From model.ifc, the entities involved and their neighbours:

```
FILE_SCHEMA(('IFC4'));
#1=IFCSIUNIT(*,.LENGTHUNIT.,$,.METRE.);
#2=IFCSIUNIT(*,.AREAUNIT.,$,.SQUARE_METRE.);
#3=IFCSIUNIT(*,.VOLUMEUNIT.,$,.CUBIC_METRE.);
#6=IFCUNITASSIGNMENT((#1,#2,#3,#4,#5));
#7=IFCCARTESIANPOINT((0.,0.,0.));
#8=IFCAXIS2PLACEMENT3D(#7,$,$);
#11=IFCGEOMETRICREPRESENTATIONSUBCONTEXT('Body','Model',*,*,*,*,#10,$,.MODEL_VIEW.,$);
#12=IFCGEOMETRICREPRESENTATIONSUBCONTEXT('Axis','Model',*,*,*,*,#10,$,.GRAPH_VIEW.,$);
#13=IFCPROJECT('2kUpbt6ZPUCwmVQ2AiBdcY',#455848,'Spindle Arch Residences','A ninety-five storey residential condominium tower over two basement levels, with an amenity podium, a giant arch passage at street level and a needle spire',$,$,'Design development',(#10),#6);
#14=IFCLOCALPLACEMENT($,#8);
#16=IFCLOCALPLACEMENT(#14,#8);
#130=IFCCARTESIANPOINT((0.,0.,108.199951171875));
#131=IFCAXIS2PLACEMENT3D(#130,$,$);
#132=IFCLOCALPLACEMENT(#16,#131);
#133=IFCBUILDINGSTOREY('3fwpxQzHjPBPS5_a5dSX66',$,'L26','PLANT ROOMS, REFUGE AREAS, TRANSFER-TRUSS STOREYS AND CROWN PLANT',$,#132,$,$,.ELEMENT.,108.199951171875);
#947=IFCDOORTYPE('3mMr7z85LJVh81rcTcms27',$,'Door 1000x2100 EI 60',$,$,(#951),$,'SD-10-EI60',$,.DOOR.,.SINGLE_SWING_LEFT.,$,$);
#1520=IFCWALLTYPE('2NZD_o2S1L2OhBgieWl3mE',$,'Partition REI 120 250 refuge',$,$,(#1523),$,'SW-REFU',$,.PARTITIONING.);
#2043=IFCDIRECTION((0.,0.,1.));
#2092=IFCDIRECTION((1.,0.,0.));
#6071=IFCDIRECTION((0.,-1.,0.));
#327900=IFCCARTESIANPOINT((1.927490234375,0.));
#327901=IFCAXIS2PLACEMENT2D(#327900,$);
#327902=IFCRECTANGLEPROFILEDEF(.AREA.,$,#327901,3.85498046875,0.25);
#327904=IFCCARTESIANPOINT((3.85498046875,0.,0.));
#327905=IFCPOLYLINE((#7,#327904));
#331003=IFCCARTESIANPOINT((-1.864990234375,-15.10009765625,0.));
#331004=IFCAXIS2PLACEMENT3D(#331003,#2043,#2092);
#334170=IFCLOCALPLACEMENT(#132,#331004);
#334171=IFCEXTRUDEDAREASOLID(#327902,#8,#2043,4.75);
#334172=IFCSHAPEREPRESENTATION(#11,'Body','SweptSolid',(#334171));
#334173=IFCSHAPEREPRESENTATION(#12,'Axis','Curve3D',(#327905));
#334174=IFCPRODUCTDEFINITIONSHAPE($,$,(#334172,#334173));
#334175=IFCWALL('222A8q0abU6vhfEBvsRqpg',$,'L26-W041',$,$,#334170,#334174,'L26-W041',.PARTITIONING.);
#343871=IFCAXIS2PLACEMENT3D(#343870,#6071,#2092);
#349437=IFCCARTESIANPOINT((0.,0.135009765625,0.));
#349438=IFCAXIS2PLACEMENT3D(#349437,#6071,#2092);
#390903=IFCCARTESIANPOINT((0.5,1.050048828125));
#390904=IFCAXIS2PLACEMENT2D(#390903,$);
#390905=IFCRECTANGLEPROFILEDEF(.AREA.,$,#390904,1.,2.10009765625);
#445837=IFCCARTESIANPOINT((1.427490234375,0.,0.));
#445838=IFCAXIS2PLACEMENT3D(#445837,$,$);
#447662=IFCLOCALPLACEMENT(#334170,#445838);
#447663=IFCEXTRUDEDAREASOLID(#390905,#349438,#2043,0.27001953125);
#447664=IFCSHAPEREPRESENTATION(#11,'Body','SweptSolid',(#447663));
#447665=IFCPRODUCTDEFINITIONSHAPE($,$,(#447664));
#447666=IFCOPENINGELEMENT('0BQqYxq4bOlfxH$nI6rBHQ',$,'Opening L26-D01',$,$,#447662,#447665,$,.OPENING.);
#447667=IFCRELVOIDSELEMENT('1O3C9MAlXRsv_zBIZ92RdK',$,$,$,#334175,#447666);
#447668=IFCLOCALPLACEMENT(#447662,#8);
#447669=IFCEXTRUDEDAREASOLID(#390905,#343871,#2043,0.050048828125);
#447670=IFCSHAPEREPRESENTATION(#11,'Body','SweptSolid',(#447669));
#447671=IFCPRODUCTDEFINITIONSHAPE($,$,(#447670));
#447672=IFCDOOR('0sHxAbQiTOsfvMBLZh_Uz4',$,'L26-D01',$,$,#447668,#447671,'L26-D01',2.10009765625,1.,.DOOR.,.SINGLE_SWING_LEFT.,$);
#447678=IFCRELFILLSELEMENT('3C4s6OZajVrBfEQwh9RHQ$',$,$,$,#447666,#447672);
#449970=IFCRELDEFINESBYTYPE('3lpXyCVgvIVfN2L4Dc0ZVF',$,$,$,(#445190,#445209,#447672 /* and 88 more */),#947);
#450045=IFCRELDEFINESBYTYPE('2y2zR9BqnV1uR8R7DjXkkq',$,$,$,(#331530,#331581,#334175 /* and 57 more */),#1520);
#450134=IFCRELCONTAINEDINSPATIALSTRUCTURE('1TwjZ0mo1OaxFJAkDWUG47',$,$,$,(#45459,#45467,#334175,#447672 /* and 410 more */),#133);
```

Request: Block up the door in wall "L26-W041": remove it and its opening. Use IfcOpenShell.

```python
import ifcopenshell
import ifcopenshell.api.feature
import ifcopenshell.api.root
import ifcopenshell.geom
import ifcopenshell.util.shape

model = ifcopenshell.open("model.ifc")
settings = ifcopenshell.geom.settings()


def volume(element):
    """Net volume in cubic metres, openings subtracted."""
    shape = ifcopenshell.geom.create_shape(settings, element)
    return ifcopenshell.util.shape.get_volume(shape.geometry)


door = model.by_id(447672)
opening = door.FillsVoids[0].RelatingOpeningElement
wall = opening.VoidsElements[0].RelatingBuildingElement
before = volume(wall)

ifcopenshell.api.root.remove_product(model, product=door)
ifcopenshell.api.feature.remove_feature(model, feature=opening)

after = volume(wall)

print(f"wall volume {before:.3f} -> {after:.3f} m3")

model.write("model-out.ifc")
```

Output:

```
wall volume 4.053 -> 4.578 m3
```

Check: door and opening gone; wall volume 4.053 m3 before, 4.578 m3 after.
